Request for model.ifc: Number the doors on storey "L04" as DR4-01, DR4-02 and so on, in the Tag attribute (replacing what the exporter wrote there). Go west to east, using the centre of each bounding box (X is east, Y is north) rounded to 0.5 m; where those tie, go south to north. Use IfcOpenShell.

First a look at what the model holds.

```python
import ifcopenshell
import ifcopenshell.util.element
import ifcopenshell.util.placement

model = ifcopenshell.open("model.ifc")
print(model.schema)
storey = next(s for s in model.by_type("IfcBuildingStorey") if s.Name == "L04")
doors = [e for e in ifcopenshell.util.element.get_decomposition(storey) if e.is_a("IfcDoor")]
for e in sorted(doors, key=lambda e: e.id()):
    origin = ifcopenshell.util.placement.get_local_placement(e.ObjectPlacement)[:3, 3]
    print(e.id(), e.Tag, e.Name, origin.round(2) + 0.0, sep=" | ")
```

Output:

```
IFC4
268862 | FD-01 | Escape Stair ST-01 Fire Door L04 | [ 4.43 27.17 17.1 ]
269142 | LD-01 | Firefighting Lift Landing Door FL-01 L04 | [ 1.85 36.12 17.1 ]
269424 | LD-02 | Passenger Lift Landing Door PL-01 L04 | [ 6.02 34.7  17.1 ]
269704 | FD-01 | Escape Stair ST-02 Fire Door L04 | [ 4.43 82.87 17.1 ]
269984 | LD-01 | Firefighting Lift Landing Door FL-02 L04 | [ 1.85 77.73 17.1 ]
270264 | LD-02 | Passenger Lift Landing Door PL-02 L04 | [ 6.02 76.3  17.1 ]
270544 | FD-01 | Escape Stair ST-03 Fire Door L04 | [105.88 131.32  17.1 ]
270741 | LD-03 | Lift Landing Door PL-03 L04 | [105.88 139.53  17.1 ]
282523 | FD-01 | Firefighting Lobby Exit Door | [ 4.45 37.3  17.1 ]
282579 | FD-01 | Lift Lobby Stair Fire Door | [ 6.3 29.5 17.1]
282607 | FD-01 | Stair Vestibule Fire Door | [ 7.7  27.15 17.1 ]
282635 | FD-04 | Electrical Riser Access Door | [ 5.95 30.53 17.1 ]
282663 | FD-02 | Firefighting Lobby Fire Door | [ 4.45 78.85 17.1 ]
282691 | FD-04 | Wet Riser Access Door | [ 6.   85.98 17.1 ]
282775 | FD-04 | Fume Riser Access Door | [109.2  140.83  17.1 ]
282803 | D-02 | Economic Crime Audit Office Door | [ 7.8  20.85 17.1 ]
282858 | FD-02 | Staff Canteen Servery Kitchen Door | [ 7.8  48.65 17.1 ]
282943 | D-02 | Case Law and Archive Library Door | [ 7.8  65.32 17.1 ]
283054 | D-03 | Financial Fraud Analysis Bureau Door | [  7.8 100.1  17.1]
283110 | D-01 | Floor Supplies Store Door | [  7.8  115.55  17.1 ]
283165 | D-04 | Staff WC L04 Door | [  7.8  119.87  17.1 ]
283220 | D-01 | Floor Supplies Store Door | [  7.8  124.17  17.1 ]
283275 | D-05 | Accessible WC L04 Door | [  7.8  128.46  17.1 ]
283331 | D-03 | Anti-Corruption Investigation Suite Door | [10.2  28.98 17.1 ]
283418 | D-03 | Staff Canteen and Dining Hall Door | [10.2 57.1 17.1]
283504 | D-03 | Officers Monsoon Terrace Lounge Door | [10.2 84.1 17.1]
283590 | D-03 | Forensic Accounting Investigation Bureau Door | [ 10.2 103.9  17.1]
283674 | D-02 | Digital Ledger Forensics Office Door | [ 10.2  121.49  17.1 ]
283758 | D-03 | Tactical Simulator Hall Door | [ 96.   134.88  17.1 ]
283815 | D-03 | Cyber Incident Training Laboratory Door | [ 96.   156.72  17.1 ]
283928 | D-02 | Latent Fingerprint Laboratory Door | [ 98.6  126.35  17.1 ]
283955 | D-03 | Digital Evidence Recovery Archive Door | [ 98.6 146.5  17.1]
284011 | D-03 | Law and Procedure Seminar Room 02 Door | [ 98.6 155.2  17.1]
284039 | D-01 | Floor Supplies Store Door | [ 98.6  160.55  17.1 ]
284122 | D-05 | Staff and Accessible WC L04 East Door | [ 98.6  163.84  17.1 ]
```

```python
import ifcopenshell
import ifcopenshell.geom
import ifcopenshell.util.element
import ifcopenshell.util.shape

model = ifcopenshell.open("model.ifc")
settings = ifcopenshell.geom.settings()
settings.set("use-world-coords", True)


def centre(element):
    shape = ifcopenshell.geom.create_shape(settings, element)
    return ifcopenshell.util.shape.get_bbox_centroid(shape.geometry)


storey = next(s for s in model.by_type("IfcBuildingStorey") if s.Name == "L04")
doors = [e for e in ifcopenshell.util.element.get_decomposition(storey) if e.is_a("IfcDoor")]

# Insertion points can sit at a corner or the storey origin, so sort by the geometry (in metres).
centres = {e: centre(e) for e in doors}
doors.sort(key=lambda e: (round(centres[e][0] / 0.5), centres[e][1]))

for i, e in enumerate(doors, start=1):
    number = f"DR4-{i:02d}"
    e.Tag = number
    print(e.id(), number)

model.write("model_rev.ifc")
```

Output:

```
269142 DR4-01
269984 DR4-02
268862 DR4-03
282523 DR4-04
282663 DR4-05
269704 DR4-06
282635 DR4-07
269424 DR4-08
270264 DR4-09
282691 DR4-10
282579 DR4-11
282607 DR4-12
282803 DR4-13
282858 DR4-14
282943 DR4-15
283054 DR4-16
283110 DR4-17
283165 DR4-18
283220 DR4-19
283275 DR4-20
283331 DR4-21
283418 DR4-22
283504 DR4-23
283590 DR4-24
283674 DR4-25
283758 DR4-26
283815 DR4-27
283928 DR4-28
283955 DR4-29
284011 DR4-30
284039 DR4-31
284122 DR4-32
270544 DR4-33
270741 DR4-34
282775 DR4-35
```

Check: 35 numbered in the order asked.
